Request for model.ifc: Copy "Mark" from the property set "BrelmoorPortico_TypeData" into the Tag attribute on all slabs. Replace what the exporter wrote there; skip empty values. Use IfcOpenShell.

First a look at what the model holds.

```python
import ifcopenshell
import ifcopenshell.util.element

model = ifcopenshell.open("model.ifc")
print(model.schema)
slabs = model.by_type("IfcSlab")
print(len(slabs), "slabs")
for e in slabs[:8]:
    source = ifcopenshell.util.element.get_pset(e, "BrelmoorPortico_TypeData", "Mark")
    target = e.Tag
    print(e.id(), repr(source), repr(target), sep=" | ")
```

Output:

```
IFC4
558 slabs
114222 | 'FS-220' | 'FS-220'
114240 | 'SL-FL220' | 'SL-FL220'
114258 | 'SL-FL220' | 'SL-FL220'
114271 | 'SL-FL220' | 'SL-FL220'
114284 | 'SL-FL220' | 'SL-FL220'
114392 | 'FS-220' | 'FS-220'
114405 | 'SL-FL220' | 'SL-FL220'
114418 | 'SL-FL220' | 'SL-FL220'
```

```python
import ifcopenshell
import ifcopenshell.util.element

model = ifcopenshell.open("model.ifc")

count = 0
for e in model.by_type("IfcSlab"):
    value = ifcopenshell.util.element.get_pset(e, "BrelmoorPortico_TypeData", "Mark")
    current = e.Tag
    if not value or not value.strip() or current == value:
        continue
    e.Tag = value
    count += 1

print(count, "slabs updated")

model.write("model_v2.ifc")
```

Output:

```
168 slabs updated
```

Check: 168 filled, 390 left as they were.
